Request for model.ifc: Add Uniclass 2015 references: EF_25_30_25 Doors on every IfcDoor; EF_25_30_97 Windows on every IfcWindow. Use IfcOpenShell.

First a look at what the model holds.

```python
import ifcopenshell

model = ifcopenshell.open("model.ifc")
print(model.schema)
print("classifications:", [c.Name for c in model.by_type("IfcClassification")])
for ifc_class in ("IfcDoor", "IfcRoof", "IfcStair", "IfcWall", "IfcWindow"):
    print(ifc_class, len(model.by_type(ifc_class)))
```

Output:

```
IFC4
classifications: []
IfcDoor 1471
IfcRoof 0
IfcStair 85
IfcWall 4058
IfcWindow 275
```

```python
import ifcopenshell
import ifcopenshell.api.classification

model = ifcopenshell.open("model.ifc")

system = ifcopenshell.api.classification.add_classification(model, classification="Uniclass 2015")

codes = {
    "IfcDoor": ("EF_25_30_25", "Doors"),
    "IfcWindow": ("EF_25_30_97", "Windows"),
}
for ifc_class, (code, name) in codes.items():
    products = model.by_type(ifc_class)
    ifcopenshell.api.classification.add_reference(
        model, products=products, classification=system, identification=code, name=name
    )
    print(code, len(products))

model.write("model_edited.ifc")
```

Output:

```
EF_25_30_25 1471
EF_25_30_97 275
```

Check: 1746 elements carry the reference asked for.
